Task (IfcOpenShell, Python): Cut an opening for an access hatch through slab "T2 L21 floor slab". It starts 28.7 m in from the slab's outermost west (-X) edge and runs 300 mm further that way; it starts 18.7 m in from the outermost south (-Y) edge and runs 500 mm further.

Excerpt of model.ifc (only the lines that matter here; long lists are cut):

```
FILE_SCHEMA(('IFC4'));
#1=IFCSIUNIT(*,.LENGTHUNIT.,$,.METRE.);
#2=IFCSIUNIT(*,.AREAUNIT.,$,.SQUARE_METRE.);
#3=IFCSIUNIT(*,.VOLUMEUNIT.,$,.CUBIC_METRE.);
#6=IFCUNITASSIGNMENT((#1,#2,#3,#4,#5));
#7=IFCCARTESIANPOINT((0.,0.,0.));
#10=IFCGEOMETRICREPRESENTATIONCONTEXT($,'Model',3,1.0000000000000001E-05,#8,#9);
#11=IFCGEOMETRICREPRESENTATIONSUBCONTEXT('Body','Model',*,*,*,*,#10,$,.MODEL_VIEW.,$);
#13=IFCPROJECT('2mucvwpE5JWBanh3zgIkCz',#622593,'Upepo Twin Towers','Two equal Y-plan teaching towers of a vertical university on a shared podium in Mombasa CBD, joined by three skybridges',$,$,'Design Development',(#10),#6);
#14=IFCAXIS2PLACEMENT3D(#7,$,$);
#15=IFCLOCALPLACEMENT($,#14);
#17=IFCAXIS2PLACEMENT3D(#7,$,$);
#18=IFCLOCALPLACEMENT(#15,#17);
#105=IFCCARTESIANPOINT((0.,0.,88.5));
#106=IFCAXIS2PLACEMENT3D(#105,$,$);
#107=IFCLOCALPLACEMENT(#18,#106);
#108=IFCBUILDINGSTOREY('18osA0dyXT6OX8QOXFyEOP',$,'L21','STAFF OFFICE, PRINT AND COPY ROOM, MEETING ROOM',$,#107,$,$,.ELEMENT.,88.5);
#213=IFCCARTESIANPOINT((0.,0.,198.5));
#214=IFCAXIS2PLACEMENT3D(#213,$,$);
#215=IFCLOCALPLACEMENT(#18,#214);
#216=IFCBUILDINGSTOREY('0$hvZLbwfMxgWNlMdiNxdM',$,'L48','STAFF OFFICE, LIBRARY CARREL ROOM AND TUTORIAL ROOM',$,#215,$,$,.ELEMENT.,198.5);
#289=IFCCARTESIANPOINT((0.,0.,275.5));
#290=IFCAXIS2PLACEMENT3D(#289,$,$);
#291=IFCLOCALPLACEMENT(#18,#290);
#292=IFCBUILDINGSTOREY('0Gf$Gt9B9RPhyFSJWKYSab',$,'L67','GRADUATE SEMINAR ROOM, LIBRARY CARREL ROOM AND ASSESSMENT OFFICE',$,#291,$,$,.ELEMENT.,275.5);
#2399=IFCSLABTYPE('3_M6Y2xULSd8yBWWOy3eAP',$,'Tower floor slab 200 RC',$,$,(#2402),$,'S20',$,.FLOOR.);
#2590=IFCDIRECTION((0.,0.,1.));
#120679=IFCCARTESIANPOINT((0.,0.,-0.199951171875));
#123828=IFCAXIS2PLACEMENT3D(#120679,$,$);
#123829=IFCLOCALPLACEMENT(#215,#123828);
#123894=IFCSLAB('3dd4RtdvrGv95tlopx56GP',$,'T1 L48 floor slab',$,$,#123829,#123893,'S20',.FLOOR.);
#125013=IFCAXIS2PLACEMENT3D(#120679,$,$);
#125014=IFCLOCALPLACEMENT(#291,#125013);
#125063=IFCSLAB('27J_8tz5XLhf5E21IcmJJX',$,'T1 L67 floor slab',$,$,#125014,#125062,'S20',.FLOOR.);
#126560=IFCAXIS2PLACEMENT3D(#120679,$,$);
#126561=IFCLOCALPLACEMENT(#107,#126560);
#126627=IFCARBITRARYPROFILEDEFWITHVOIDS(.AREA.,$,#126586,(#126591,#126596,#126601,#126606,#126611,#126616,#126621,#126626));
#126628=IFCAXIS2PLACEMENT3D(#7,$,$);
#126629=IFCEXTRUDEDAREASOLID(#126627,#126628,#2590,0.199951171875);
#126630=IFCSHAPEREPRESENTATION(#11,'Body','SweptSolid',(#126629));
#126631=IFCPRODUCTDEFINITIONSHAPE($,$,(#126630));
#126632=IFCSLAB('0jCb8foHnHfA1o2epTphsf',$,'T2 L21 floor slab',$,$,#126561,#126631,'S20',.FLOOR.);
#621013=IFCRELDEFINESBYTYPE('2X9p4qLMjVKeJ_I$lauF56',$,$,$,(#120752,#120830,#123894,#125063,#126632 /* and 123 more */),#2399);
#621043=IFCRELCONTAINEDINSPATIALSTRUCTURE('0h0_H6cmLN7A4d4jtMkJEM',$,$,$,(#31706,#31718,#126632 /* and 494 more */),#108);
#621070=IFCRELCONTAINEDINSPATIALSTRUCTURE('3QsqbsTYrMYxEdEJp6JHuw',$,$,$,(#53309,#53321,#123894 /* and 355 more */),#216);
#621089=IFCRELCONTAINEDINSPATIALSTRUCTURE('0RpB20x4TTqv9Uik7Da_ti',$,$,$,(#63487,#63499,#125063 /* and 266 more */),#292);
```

```python
import numpy as np
import ifcopenshell
import ifcopenshell.api.feature
import ifcopenshell.api.geometry
import ifcopenshell.api.root
import ifcopenshell.geom
import ifcopenshell.util.placement
import ifcopenshell.util.representation
import ifcopenshell.util.shape
import ifcopenshell.util.unit

model = ifcopenshell.open("model.ifc")
unit_scale = ifcopenshell.util.unit.calculate_unit_scale(model)
settings = ifcopenshell.geom.settings()


def volume(element):
    """Net volume in cubic metres, openings subtracted."""
    shape = ifcopenshell.geom.create_shape(settings, element)
    return ifcopenshell.util.shape.get_volume(shape.geometry)


slab = model.by_guid("0jCb8foHnHfA1o2epTphsf")
before = volume(slab)

# Extent in the slab's own axes, in metres. The edges named are its -X and -Y sides.
slab_shape = ifcopenshell.geom.create_shape(settings, slab)
vertices = ifcopenshell.util.shape.get_vertices(slab_shape.geometry)
x_min, y_min, bottom = vertices.min(axis=0)
top = vertices[:, 2].max()

opening = ifcopenshell.api.root.create_entity(model, ifc_class="IfcOpeningElement", name="Access hatch opening", predefined_type="OPENING")
context = ifcopenshell.util.representation.get_context(model, "Model", "Body", "MODEL_VIEW")
width, depth = 0.3, 0.5
outline = [(0.0, 0.0), (width, 0.0), (width, depth), (0.0, depth), (0.0, 0.0)]
# Overshoot both faces by 50 mm so the cut is clean.
shape = ifcopenshell.api.geometry.add_slab_representation(
    model, context=context, depth=top - bottom + 0.1, polyline=outline
)
ifcopenshell.api.geometry.assign_representation(model, product=opening, representation=shape)

matrix = ifcopenshell.util.placement.get_local_placement(slab.ObjectPlacement)
matrix[:, 3] = matrix @ np.append(np.array([x_min + 28.7, y_min + 18.7, bottom - 0.05]) / unit_scale, 1.0)
ifcopenshell.api.geometry.edit_object_placement(model, product=opening, matrix=matrix, is_si=False)
ifcopenshell.api.feature.add_feature(model, feature=opening, element=slab)

after = volume(slab)

print(f"slab volume {before:.3f} -> {after:.3f} m3")

model.write("model_edited.ifc")
```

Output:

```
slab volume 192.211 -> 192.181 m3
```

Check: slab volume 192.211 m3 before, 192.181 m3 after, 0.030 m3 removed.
